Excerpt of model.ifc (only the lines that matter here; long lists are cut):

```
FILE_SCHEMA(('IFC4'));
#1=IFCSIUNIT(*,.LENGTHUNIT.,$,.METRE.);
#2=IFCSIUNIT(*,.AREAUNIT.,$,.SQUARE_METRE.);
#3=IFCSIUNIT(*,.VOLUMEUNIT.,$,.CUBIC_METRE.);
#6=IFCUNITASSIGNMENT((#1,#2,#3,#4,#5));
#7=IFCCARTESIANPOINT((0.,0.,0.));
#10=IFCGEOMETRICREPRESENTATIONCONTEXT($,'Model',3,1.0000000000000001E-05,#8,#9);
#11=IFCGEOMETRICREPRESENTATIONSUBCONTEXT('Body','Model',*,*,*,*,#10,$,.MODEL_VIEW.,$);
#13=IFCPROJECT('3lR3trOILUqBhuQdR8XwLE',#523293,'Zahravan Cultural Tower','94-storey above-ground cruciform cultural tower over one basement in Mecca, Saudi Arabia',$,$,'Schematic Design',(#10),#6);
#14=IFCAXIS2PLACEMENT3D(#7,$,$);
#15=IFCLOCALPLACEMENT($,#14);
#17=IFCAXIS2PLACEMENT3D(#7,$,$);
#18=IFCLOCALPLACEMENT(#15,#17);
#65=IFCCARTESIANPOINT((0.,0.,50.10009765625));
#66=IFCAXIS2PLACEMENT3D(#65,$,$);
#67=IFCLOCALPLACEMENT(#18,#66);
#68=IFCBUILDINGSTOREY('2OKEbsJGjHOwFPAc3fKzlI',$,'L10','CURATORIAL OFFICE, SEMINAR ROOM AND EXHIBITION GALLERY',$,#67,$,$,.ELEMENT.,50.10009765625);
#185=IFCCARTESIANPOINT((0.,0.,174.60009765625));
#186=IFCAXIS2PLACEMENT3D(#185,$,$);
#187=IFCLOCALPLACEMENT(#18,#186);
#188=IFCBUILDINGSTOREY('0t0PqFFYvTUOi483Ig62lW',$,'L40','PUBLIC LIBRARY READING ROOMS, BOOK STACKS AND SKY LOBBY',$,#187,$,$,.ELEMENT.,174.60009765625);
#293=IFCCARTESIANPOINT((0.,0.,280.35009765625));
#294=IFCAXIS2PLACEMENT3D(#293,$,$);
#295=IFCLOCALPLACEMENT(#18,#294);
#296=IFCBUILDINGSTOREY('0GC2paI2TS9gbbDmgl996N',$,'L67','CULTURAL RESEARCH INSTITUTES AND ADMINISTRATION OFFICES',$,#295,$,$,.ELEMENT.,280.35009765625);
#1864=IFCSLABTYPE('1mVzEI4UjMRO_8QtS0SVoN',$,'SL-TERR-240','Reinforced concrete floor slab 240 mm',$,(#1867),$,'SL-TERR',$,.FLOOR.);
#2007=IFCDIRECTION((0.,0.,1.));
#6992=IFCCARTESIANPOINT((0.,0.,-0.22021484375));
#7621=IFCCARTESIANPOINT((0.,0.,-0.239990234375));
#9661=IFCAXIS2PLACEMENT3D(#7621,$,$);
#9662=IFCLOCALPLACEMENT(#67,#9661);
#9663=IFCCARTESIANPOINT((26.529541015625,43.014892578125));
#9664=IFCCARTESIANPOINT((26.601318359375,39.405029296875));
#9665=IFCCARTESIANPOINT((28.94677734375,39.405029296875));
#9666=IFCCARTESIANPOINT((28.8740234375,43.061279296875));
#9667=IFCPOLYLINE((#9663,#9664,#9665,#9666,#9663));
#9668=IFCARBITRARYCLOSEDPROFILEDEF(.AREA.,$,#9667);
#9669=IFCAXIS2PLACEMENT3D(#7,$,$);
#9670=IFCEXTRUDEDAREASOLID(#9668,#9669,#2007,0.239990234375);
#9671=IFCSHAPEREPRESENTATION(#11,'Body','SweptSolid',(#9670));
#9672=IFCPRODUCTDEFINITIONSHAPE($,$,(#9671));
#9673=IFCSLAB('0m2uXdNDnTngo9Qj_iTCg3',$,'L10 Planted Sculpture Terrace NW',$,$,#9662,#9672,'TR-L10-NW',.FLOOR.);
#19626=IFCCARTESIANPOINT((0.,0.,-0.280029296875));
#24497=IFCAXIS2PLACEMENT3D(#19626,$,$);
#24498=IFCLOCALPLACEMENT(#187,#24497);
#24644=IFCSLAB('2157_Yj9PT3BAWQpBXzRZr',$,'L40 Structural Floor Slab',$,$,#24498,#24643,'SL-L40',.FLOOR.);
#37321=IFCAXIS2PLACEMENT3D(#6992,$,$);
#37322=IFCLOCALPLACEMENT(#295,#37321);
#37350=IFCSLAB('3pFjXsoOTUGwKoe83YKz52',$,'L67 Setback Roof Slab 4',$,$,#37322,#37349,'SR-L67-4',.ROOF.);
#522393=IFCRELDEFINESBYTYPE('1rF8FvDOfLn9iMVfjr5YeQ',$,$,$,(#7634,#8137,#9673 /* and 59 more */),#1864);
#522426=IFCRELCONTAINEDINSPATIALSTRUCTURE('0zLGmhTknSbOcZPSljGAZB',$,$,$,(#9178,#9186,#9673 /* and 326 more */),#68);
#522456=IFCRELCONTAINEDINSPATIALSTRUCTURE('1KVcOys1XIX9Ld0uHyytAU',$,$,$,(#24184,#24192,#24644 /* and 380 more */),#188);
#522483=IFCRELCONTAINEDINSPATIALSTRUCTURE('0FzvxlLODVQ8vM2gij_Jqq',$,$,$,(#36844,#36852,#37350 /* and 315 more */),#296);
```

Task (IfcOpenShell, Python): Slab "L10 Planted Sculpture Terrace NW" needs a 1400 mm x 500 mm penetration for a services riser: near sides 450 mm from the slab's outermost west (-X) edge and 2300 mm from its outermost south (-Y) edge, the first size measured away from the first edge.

```python
import numpy as np
import ifcopenshell
import ifcopenshell.api.feature
import ifcopenshell.api.geometry
import ifcopenshell.api.root
import ifcopenshell.geom
import ifcopenshell.util.placement
import ifcopenshell.util.representation
import ifcopenshell.util.shape
import ifcopenshell.util.unit

model = ifcopenshell.open("model.ifc")
unit_scale = ifcopenshell.util.unit.calculate_unit_scale(model)
settings = ifcopenshell.geom.settings()


def volume(element):
    """Net volume in cubic metres, openings subtracted."""
    shape = ifcopenshell.geom.create_shape(settings, element)
    return ifcopenshell.util.shape.get_volume(shape.geometry)


slab = model.by_guid("0m2uXdNDnTngo9Qj_iTCg3")
before = volume(slab)

# Extent in the slab's own axes, in metres. The edges named are its -X and -Y sides.
slab_shape = ifcopenshell.geom.create_shape(settings, slab)
vertices = ifcopenshell.util.shape.get_vertices(slab_shape.geometry)
x_min, y_min, bottom = vertices.min(axis=0)
top = vertices[:, 2].max()

opening = ifcopenshell.api.root.create_entity(model, ifc_class="IfcOpeningElement", name="Services riser opening", predefined_type="OPENING")
context = ifcopenshell.util.representation.get_context(model, "Model", "Body", "MODEL_VIEW")
width, depth = 1.4, 0.5
outline = [(0.0, 0.0), (width, 0.0), (width, depth), (0.0, depth), (0.0, 0.0)]
# Overshoot both faces by 50 mm so the cut is clean.
shape = ifcopenshell.api.geometry.add_slab_representation(
    model, context=context, depth=top - bottom + 0.1, polyline=outline
)
ifcopenshell.api.geometry.assign_representation(model, product=opening, representation=shape)

matrix = ifcopenshell.util.placement.get_local_placement(slab.ObjectPlacement)
matrix[:, 3] = matrix @ np.append(np.array([x_min + 0.45, y_min + 2.3, bottom - 0.05]) / unit_scale, 1.0)
ifcopenshell.api.geometry.edit_object_placement(model, product=opening, matrix=matrix, is_si=False)
ifcopenshell.api.feature.add_feature(model, feature=opening, element=slab)

after = volume(slab)

print(f"slab volume {before:.3f} -> {after:.3f} m3")

model.write("model-out.ifc")
```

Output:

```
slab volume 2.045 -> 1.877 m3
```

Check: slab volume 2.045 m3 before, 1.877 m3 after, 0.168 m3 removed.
